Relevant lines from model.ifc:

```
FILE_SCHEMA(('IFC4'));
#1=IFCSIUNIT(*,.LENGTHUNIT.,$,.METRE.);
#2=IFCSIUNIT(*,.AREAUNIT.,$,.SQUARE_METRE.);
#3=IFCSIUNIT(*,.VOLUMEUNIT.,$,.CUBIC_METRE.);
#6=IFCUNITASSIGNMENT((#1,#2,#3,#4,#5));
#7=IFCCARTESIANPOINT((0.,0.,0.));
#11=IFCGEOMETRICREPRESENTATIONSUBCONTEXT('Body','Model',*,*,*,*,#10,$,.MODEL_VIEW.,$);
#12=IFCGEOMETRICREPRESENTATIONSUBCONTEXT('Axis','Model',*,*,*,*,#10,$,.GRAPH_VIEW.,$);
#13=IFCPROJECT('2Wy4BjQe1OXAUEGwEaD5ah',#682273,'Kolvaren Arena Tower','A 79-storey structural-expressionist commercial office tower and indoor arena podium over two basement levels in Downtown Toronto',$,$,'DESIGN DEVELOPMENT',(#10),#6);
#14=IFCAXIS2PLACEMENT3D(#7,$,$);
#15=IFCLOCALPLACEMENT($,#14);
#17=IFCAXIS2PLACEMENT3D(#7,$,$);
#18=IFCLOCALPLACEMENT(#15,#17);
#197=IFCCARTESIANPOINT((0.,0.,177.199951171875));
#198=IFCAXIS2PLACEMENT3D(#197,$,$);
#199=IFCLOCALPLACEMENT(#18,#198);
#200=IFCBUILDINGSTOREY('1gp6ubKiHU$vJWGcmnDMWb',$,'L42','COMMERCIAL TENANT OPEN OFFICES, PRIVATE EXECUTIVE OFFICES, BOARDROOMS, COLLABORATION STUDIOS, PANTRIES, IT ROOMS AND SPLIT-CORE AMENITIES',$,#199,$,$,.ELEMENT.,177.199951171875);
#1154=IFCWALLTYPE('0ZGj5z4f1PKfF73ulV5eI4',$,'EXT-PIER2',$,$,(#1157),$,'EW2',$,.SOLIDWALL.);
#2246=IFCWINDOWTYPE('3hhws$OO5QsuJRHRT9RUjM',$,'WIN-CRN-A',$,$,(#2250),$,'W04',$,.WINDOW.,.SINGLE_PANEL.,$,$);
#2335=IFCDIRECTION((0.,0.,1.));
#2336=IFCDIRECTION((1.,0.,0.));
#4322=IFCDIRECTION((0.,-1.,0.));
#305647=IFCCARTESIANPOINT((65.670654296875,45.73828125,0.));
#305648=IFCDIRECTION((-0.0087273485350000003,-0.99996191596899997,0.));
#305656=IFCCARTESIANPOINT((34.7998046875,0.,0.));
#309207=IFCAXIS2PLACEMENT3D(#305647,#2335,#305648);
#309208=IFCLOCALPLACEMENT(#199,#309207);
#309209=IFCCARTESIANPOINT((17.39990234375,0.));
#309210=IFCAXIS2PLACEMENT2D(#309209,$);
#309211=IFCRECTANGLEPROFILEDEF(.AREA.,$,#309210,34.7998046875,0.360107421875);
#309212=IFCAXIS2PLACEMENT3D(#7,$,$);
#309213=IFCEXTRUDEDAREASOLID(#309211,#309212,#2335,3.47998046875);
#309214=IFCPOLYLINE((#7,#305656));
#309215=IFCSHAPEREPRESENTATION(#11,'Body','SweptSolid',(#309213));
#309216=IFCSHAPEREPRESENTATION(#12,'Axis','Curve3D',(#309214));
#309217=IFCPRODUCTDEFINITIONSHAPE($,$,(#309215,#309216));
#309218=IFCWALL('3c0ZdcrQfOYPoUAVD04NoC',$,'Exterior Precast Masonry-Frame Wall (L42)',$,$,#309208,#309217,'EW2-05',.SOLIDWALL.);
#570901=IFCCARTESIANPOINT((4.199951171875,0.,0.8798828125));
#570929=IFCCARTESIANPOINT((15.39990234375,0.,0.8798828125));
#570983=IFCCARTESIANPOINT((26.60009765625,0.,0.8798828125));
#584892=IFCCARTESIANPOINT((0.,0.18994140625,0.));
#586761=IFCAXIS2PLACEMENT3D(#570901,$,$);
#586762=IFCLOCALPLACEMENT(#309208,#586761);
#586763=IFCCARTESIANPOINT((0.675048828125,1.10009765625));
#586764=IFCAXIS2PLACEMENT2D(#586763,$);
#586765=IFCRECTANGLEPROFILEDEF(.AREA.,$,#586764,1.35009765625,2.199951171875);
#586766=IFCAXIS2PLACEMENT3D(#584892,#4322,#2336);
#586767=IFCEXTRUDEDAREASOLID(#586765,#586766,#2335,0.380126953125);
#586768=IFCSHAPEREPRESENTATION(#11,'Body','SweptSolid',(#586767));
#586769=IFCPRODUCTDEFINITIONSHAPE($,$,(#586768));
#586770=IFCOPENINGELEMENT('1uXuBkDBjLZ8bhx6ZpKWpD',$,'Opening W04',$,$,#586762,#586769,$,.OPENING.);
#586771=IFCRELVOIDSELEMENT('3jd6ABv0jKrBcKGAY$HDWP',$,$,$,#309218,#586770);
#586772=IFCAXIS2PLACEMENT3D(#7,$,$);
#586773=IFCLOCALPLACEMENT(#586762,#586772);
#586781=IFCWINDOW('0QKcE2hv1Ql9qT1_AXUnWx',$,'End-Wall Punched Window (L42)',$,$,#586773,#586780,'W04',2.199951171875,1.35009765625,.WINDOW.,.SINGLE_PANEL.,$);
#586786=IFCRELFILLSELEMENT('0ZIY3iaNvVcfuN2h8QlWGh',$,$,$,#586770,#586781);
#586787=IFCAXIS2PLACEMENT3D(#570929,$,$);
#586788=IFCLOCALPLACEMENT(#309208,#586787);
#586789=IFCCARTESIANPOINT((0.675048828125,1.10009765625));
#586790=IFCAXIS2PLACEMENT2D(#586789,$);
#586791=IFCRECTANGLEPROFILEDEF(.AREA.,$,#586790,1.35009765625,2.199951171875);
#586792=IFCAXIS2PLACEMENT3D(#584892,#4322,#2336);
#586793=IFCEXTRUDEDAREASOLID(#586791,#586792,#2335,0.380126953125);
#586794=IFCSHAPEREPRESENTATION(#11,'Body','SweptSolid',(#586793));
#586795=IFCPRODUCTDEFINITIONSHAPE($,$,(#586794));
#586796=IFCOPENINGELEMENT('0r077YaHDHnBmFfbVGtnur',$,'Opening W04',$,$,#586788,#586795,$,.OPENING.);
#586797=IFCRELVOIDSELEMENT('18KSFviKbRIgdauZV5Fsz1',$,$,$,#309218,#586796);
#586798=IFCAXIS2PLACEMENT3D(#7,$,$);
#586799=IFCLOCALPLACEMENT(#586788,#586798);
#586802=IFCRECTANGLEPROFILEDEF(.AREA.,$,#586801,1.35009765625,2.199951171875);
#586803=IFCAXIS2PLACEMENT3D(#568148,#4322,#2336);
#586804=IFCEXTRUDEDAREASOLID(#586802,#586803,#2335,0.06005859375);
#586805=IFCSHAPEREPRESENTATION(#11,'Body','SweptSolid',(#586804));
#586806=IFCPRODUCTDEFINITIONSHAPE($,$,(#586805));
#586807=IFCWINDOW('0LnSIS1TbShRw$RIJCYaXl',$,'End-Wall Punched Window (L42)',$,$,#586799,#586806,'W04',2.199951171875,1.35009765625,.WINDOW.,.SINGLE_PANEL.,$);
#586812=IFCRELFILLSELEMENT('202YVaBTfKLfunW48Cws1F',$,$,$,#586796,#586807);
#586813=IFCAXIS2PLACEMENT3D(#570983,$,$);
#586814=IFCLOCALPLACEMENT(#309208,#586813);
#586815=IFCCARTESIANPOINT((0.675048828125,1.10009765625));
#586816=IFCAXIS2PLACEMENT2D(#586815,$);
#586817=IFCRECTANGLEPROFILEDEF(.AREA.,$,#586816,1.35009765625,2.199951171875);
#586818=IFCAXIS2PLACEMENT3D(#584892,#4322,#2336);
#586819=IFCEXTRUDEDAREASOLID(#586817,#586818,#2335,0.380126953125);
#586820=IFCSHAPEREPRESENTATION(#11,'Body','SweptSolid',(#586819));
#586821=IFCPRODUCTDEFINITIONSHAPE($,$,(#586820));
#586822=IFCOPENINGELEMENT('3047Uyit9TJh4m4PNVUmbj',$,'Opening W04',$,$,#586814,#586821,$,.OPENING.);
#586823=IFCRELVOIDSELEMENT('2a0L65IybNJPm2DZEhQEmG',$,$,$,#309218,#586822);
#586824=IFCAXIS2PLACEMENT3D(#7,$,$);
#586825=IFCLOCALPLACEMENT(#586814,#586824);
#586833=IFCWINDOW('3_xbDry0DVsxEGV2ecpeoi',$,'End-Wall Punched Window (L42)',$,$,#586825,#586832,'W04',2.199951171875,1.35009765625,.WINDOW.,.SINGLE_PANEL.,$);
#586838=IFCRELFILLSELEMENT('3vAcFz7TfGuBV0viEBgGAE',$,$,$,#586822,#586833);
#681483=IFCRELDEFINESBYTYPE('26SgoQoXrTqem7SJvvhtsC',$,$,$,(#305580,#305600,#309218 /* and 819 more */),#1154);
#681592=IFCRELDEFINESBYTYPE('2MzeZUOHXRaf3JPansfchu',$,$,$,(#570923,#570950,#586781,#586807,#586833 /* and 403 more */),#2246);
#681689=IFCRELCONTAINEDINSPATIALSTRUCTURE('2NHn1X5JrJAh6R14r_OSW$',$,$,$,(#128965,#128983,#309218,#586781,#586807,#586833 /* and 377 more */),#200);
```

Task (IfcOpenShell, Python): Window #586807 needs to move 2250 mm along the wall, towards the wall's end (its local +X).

```python
import ifcopenshell
import ifcopenshell.api.geometry
import ifcopenshell.util.placement

model = ifcopenshell.open("model.ifc")

window = model.by_guid("0LnSIS1TbShRw$RIJCYaXl")
opening = window.FillsVoids[0].RelatingOpeningElement
wall = opening.VoidsElements[0].RelatingBuildingElement

wall_matrix = ifcopenshell.util.placement.get_local_placement(wall.ObjectPlacement)
shift = wall_matrix[:3, 0] * 2.25
before = ifcopenshell.util.placement.get_local_placement(window.ObjectPlacement)[:3, 3].copy()

# The window is placed relative to its opening, so it follows when the opening moves.
matrix = ifcopenshell.util.placement.get_local_placement(opening.ObjectPlacement)
matrix[:3, 3] += shift
ifcopenshell.api.geometry.edit_object_placement(
    model, product=opening, matrix=matrix, is_si=False, should_transform_children=True
)

after = ifcopenshell.util.placement.get_local_placement(window.ObjectPlacement)[:3, 3]
print("window moved by", (after - before).round(3) + 0.0)

model.write("model_v2.ifc")
```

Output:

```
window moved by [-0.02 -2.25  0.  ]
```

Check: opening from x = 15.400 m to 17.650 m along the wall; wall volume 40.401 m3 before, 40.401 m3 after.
